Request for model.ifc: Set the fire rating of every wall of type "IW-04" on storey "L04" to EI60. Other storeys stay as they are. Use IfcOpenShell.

First a look at what the model holds.

```python
import ifcopenshell
import ifcopenshell.util.element

model = ifcopenshell.open("model.ifc")
print(model.schema)
storey = next(s for s in model.by_type("IfcBuildingStorey") if s.Name == "L04")
walls = [e for e in ifcopenshell.util.element.get_decomposition(storey) if e.is_a("IfcWall")]
seen = {}
for e in walls:
    element_type = ifcopenshell.util.element.get_type(e)
    key = (element_type.Name if element_type != e and element_type else None, ifcopenshell.util.element.get_pset(e, "Pset_WallCommon", "FireRating"))
    seen[key] = seen.get(key, 0) + 1
for (name, value), count in sorted(seen.items(), key=str):
    print(count, "x", name, "|", value)
```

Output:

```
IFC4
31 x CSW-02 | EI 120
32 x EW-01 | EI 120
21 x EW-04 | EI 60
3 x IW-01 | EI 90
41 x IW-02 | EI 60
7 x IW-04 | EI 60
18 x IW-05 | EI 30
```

```python
import ifcopenshell
import ifcopenshell.api.pset
import ifcopenshell.util.element

model = ifcopenshell.open("model.ifc")

storey = next(s for s in model.by_type("IfcBuildingStorey") if s.Name == "L04")
walls = [e for e in ifcopenshell.util.element.get_decomposition(storey) if e.is_a("IfcWall")]

count = 0
for e in walls:
    element_type = ifcopenshell.util.element.get_type(e)
    if element_type in (None, e) or element_type.Name != "IW-04":
        continue
    # add_pset returns the element's existing set when there is one.
    pset = ifcopenshell.api.pset.add_pset(model, product=e, name="Pset_WallCommon")
    ifcopenshell.api.pset.edit_pset(model, pset=pset, properties={"FireRating": "EI60"})
    count += 1

print(count, "walls updated")

model.write("model-out.ifc")
```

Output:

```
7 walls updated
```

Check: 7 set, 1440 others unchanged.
